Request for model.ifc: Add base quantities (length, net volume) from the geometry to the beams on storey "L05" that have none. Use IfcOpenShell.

First a look at what the model holds.

```python
import ifcopenshell
import ifcopenshell.util.element
import ifcopenshell.util.unit

model = ifcopenshell.open("model.ifc")
print(model.schema)
for unit_type in ("LENGTHUNIT", "AREAUNIT", "VOLUMEUNIT"):
    print(unit_type, ifcopenshell.util.unit.calculate_unit_scale(model, unit_type))
storey = next(s for s in model.by_type("IfcBuildingStorey") if s.Name == "L05")
beams = [e for e in ifcopenshell.util.element.get_decomposition(storey) if e.is_a("IfcBeam")]
for e in sorted(beams, key=lambda e: e.id()):
    print(e.id(), e.is_a(), e.Name, list(ifcopenshell.util.element.get_psets(e, qtos_only=True)), sep=" | ")
```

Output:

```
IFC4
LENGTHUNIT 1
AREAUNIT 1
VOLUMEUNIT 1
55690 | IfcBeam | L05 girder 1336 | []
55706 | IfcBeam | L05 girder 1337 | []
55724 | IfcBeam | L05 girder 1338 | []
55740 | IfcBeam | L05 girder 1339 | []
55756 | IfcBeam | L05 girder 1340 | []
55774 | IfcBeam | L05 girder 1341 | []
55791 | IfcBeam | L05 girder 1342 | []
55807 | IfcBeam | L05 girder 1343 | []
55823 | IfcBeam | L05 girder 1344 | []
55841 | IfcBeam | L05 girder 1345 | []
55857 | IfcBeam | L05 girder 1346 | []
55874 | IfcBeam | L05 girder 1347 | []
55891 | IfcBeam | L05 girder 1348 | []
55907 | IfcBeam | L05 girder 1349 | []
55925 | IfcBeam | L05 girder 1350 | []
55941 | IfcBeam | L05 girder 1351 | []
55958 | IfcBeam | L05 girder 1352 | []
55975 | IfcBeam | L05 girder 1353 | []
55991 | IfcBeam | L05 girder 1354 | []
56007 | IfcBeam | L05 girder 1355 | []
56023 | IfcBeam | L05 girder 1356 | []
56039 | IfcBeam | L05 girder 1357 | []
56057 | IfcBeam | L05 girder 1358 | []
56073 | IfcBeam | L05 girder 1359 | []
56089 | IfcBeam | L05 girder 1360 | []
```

```python
import ifcopenshell
import ifcopenshell.api.pset
import ifcopenshell.geom
import ifcopenshell.util.element
import ifcopenshell.util.shape
import ifcopenshell.util.unit

model = ifcopenshell.open("model.ifc")
unit_scale = ifcopenshell.util.unit.calculate_unit_scale(model)
volume_scale = ifcopenshell.util.unit.calculate_unit_scale(model, "VOLUMEUNIT")
settings = ifcopenshell.geom.settings()

storey = next(s for s in model.by_type("IfcBuildingStorey") if s.Name == "L05")
beams = [e for e in ifcopenshell.util.element.get_decomposition(storey) if e.is_a("IfcBeam")]

for e in sorted(beams, key=lambda e: e.id()):
    if ifcopenshell.util.element.get_psets(e, qtos_only=True, should_inherit=False):
        continue
    # Geometry comes back in metres, in the element's own axes.
    shape = ifcopenshell.geom.create_shape(settings, e)
    values = {
        "Length": ifcopenshell.util.shape.get_max_xyz(shape.geometry) / unit_scale,
        "NetVolume": ifcopenshell.util.shape.get_volume(shape.geometry) / volume_scale,
    }
    qto = ifcopenshell.api.pset.add_qto(model, product=e, name="Qto_BeamBaseQuantities")
    ifcopenshell.api.pset.edit_qto(model, qto=qto, properties=values)
    print(e.id(), {k: round(v, 3) for k, v in values.items()})

model.write("model-out.ifc")
```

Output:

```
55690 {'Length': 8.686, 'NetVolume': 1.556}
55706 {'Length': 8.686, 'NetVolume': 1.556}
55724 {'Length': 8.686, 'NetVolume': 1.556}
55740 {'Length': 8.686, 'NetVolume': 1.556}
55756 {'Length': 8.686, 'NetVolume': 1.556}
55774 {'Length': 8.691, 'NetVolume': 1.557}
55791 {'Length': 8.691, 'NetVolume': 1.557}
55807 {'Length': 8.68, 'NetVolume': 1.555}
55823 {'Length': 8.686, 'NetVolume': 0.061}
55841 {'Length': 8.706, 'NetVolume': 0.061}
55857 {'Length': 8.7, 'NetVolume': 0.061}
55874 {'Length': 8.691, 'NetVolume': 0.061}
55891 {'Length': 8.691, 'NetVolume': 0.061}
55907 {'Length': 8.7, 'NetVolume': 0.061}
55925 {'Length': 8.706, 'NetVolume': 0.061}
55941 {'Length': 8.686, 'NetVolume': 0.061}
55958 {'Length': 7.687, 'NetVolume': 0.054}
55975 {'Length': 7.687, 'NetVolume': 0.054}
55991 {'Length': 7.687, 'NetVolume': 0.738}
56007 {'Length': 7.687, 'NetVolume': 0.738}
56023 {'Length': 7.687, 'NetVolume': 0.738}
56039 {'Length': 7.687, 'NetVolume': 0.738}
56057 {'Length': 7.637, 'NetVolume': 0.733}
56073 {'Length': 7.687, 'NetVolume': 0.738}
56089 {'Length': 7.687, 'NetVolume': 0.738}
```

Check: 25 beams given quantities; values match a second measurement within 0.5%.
